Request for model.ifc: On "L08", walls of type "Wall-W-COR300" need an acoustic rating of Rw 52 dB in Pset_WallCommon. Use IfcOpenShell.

First a look at what the model holds.

```python
import ifcopenshell
import ifcopenshell.util.element

model = ifcopenshell.open("model.ifc")
print(model.schema)
storey = next(s for s in model.by_type("IfcBuildingStorey") if s.Name == "L08")
walls = [e for e in ifcopenshell.util.element.get_decomposition(storey) if e.is_a("IfcWall")]
seen = {}
for e in walls:
    element_type = ifcopenshell.util.element.get_type(e)
    key = (element_type.Name if element_type != e and element_type else None, ifcopenshell.util.element.get_pset(e, "Pset_WallCommon", "AcousticRating"))
    seen[key] = seen.get(key, 0) + 1
for (name, value), count in sorted(seen.items(), key=str):
    print(count, "x", name, "|", value)
```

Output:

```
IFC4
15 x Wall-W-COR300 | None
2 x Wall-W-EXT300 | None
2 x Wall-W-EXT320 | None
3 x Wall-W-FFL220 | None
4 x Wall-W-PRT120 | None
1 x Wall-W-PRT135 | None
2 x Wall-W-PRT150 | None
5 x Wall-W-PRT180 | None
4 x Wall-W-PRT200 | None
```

```python
import ifcopenshell
import ifcopenshell.api.pset
import ifcopenshell.util.element

model = ifcopenshell.open("model.ifc")

storey = next(s for s in model.by_type("IfcBuildingStorey") if s.Name == "L08")
walls = [e for e in ifcopenshell.util.element.get_decomposition(storey) if e.is_a("IfcWall")]

count = 0
for e in walls:
    element_type = ifcopenshell.util.element.get_type(e)
    if element_type in (None, e) or element_type.Name != "Wall-W-COR300":
        continue
    # add_pset returns the element's existing set when there is one.
    pset = ifcopenshell.api.pset.add_pset(model, product=e, name="Pset_WallCommon")
    ifcopenshell.api.pset.edit_pset(model, pset=pset, properties={"AcousticRating": "Rw 52 dB"})
    count += 1

print(count, "walls updated")

model.write("model-out.ifc")
```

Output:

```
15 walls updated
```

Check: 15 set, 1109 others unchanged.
